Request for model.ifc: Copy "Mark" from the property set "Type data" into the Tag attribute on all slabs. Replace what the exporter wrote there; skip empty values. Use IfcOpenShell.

First a look at what the model holds.

```python
import ifcopenshell
import ifcopenshell.util.element

model = ifcopenshell.open("model.ifc")
print(model.schema)
slabs = model.by_type("IfcSlab")
print(len(slabs), "slabs")
for e in slabs[:8]:
    source = ifcopenshell.util.element.get_pset(e, "Type data", "Mark")
    target = e.Tag
    print(e.id(), repr(source), repr(target), sep=" | ")
```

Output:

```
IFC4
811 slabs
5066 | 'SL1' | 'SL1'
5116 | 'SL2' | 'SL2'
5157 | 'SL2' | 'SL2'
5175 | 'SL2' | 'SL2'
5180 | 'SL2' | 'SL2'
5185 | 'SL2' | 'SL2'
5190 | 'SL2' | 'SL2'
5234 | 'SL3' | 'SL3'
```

```python
import ifcopenshell
import ifcopenshell.util.element

model = ifcopenshell.open("model.ifc")

count = 0
for e in model.by_type("IfcSlab"):
    value = ifcopenshell.util.element.get_pset(e, "Type data", "Mark")
    current = e.Tag
    if not value or not value.strip() or current == value:
        continue
    e.Tag = value
    count += 1

print(count, "slabs updated")

model.write("model_updated.ifc")
```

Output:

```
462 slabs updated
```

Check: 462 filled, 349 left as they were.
